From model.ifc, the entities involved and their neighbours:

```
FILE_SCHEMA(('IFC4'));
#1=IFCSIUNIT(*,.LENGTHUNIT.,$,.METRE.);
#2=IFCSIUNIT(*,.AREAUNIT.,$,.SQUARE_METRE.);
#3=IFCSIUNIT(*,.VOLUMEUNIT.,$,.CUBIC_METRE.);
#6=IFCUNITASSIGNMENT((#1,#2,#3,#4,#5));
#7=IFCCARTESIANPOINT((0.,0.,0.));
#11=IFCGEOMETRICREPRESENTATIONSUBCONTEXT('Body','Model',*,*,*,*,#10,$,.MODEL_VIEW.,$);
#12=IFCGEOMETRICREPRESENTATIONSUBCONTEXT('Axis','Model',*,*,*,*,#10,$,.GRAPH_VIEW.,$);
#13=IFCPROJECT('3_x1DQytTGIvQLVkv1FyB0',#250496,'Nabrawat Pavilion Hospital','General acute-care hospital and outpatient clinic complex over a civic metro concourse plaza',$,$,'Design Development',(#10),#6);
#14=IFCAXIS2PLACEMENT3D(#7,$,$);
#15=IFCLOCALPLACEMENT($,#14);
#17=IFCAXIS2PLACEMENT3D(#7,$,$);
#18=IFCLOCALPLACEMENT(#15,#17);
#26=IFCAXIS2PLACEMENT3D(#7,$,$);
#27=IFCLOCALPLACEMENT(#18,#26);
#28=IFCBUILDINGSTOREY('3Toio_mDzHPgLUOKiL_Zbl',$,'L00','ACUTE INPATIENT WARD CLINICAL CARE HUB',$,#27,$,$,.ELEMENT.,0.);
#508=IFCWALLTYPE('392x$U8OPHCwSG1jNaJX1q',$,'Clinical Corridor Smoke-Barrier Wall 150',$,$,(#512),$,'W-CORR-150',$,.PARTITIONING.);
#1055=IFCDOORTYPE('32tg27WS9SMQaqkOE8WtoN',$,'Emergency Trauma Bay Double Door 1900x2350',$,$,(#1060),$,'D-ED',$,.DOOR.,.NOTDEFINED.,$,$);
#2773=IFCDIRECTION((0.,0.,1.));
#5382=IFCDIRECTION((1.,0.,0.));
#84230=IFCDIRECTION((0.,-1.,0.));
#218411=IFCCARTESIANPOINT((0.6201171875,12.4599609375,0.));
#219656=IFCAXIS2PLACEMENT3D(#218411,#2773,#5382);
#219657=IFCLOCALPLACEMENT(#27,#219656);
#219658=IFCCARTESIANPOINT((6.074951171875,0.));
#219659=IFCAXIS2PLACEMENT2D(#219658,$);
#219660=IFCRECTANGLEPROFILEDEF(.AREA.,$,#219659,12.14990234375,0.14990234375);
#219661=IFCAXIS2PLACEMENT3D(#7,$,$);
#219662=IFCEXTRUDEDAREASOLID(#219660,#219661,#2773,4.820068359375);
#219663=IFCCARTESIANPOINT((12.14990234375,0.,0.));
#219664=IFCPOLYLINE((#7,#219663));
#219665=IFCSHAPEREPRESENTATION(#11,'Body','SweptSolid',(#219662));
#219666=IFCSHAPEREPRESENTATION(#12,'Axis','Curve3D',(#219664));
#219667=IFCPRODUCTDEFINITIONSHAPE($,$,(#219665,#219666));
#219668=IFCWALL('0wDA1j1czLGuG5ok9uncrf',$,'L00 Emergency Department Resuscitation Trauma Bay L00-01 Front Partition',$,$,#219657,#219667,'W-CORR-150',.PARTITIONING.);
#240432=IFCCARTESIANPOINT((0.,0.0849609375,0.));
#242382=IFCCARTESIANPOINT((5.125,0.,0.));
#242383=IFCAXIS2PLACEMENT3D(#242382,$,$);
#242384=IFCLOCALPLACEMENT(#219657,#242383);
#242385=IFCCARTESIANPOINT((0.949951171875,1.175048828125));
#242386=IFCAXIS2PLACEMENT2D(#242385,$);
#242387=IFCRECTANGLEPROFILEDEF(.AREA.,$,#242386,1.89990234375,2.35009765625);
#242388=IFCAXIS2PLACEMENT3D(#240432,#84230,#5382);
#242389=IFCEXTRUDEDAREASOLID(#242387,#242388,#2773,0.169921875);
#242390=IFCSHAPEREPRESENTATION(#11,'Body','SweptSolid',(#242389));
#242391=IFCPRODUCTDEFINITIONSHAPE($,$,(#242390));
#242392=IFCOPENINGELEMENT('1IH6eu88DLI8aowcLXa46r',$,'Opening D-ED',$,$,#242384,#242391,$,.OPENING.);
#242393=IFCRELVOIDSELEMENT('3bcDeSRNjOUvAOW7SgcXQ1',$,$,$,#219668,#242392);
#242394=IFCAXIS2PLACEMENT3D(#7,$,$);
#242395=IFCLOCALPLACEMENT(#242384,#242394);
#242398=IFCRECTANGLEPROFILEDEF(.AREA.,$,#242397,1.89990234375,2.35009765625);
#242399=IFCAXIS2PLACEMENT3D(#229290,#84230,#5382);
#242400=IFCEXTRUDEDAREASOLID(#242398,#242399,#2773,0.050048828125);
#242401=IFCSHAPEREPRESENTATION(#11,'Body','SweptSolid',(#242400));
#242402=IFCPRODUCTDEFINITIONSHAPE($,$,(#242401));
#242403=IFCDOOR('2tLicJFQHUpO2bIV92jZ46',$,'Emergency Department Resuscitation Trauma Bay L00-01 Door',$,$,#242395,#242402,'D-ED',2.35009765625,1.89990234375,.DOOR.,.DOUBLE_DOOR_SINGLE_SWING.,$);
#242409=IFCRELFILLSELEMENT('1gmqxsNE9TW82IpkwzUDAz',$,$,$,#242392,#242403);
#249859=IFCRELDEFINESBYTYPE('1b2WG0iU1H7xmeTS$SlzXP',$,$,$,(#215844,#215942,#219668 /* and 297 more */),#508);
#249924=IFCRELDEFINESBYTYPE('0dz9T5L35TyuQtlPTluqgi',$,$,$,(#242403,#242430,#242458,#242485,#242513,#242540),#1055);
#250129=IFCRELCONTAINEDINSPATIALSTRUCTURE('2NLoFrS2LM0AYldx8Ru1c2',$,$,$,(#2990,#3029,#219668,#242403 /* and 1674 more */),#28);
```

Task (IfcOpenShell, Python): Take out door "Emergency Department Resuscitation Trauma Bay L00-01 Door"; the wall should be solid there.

```python
import ifcopenshell
import ifcopenshell.api.feature
import ifcopenshell.api.root
import ifcopenshell.geom
import ifcopenshell.util.shape

model = ifcopenshell.open("model.ifc")
settings = ifcopenshell.geom.settings()


def volume(element):
    """Net volume in cubic metres, openings subtracted."""
    shape = ifcopenshell.geom.create_shape(settings, element)
    return ifcopenshell.util.shape.get_volume(shape.geometry)


door = model.by_guid("2tLicJFQHUpO2bIV92jZ46")
opening = door.FillsVoids[0].RelatingOpeningElement
wall = opening.VoidsElements[0].RelatingBuildingElement
before = volume(wall)

ifcopenshell.api.root.remove_product(model, product=door)
ifcopenshell.api.feature.remove_feature(model, feature=opening)

after = volume(wall)

print(f"wall volume {before:.3f} -> {after:.3f} m3")

model.write("model_v2.ifc")
```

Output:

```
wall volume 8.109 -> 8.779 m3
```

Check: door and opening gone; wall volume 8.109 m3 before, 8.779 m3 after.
